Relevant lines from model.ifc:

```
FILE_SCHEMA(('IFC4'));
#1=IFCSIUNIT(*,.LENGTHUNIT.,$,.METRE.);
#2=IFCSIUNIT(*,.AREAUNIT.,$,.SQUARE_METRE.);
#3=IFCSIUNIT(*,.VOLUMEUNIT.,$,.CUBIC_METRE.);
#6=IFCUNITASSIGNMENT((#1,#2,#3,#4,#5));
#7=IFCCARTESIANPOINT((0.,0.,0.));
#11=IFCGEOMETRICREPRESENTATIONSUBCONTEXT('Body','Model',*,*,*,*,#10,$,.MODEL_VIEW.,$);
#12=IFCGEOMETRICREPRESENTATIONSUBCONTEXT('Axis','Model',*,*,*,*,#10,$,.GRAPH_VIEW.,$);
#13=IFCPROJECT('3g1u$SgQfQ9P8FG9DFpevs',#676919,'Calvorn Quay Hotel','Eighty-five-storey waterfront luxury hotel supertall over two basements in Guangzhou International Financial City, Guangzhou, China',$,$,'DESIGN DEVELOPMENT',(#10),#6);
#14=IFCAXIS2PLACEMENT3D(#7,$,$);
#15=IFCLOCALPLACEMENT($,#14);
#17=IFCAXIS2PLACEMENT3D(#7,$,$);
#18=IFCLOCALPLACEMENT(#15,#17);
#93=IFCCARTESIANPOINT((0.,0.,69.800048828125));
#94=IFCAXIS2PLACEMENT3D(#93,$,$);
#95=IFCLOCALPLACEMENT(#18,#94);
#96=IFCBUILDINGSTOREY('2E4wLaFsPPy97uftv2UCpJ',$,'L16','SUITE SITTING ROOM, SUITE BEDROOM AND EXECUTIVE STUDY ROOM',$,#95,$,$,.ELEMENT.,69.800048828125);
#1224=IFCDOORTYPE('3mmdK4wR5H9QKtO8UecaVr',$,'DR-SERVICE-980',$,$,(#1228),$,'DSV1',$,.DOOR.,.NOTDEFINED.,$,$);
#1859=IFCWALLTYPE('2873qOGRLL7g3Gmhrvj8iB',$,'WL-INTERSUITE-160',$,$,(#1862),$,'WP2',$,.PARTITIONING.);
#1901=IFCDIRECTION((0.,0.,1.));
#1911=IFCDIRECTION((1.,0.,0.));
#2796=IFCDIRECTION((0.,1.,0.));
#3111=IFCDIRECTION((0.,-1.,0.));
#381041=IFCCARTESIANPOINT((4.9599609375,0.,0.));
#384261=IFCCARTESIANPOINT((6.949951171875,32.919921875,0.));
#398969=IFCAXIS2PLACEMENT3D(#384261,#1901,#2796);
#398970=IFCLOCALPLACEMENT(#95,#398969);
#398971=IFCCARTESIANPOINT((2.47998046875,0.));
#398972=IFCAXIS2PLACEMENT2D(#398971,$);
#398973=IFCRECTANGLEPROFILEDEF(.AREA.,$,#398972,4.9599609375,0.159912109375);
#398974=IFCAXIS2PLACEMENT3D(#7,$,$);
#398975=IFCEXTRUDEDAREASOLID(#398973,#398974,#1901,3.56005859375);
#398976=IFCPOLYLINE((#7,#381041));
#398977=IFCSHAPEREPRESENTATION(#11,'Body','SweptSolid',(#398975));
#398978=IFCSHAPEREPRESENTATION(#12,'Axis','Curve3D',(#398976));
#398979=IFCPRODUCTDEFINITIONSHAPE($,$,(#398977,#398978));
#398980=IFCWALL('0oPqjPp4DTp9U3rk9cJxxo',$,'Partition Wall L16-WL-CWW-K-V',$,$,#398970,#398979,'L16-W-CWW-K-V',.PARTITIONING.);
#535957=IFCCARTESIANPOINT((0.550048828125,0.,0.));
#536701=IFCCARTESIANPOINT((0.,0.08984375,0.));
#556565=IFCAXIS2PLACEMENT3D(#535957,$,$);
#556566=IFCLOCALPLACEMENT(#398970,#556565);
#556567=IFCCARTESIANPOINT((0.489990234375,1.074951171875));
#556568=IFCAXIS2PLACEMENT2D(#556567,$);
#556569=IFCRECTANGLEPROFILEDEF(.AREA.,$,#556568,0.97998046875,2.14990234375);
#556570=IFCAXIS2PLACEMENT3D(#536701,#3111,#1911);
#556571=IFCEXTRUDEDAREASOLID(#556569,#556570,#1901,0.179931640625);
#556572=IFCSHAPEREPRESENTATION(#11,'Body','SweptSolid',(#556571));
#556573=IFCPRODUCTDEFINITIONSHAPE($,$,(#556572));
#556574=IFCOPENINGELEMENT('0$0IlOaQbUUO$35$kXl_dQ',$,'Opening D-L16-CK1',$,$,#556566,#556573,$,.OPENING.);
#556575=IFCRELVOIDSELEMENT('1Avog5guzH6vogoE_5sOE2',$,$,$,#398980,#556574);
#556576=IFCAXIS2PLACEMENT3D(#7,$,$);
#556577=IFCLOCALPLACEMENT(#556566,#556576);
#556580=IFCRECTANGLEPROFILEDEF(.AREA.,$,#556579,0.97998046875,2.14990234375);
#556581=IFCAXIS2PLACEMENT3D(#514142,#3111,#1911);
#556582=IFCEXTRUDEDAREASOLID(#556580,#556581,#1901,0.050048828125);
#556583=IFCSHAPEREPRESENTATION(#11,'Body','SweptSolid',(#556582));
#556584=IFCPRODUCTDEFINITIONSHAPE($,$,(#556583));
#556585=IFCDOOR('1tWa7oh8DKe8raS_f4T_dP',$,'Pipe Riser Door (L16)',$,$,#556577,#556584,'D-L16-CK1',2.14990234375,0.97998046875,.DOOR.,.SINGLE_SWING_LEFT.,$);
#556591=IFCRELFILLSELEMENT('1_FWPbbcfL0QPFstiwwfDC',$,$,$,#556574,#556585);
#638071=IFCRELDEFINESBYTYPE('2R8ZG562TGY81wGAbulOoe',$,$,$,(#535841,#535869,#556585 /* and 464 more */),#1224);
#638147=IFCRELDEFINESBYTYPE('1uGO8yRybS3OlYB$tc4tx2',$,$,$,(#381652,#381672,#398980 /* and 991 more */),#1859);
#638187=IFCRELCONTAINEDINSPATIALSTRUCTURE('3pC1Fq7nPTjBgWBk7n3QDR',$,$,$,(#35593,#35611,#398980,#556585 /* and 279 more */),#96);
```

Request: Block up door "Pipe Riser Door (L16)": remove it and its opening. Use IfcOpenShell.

```python
import ifcopenshell
import ifcopenshell.api.feature
import ifcopenshell.api.root
import ifcopenshell.geom
import ifcopenshell.util.shape

model = ifcopenshell.open("model.ifc")
settings = ifcopenshell.geom.settings()


def volume(element):
    """Net volume in cubic metres, openings subtracted."""
    shape = ifcopenshell.geom.create_shape(settings, element)
    return ifcopenshell.util.shape.get_volume(shape.geometry)


door = model.by_guid("1tWa7oh8DKe8raS_f4T_dP")
opening = door.FillsVoids[0].RelatingOpeningElement
wall = opening.VoidsElements[0].RelatingBuildingElement
before = volume(wall)

ifcopenshell.api.root.remove_product(model, product=door)
ifcopenshell.api.feature.remove_feature(model, feature=opening)

after = volume(wall)

print(f"wall volume {before:.3f} -> {after:.3f} m3")

model.write("model_rev.ifc")
```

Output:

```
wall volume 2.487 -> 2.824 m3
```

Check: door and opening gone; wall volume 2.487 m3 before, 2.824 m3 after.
